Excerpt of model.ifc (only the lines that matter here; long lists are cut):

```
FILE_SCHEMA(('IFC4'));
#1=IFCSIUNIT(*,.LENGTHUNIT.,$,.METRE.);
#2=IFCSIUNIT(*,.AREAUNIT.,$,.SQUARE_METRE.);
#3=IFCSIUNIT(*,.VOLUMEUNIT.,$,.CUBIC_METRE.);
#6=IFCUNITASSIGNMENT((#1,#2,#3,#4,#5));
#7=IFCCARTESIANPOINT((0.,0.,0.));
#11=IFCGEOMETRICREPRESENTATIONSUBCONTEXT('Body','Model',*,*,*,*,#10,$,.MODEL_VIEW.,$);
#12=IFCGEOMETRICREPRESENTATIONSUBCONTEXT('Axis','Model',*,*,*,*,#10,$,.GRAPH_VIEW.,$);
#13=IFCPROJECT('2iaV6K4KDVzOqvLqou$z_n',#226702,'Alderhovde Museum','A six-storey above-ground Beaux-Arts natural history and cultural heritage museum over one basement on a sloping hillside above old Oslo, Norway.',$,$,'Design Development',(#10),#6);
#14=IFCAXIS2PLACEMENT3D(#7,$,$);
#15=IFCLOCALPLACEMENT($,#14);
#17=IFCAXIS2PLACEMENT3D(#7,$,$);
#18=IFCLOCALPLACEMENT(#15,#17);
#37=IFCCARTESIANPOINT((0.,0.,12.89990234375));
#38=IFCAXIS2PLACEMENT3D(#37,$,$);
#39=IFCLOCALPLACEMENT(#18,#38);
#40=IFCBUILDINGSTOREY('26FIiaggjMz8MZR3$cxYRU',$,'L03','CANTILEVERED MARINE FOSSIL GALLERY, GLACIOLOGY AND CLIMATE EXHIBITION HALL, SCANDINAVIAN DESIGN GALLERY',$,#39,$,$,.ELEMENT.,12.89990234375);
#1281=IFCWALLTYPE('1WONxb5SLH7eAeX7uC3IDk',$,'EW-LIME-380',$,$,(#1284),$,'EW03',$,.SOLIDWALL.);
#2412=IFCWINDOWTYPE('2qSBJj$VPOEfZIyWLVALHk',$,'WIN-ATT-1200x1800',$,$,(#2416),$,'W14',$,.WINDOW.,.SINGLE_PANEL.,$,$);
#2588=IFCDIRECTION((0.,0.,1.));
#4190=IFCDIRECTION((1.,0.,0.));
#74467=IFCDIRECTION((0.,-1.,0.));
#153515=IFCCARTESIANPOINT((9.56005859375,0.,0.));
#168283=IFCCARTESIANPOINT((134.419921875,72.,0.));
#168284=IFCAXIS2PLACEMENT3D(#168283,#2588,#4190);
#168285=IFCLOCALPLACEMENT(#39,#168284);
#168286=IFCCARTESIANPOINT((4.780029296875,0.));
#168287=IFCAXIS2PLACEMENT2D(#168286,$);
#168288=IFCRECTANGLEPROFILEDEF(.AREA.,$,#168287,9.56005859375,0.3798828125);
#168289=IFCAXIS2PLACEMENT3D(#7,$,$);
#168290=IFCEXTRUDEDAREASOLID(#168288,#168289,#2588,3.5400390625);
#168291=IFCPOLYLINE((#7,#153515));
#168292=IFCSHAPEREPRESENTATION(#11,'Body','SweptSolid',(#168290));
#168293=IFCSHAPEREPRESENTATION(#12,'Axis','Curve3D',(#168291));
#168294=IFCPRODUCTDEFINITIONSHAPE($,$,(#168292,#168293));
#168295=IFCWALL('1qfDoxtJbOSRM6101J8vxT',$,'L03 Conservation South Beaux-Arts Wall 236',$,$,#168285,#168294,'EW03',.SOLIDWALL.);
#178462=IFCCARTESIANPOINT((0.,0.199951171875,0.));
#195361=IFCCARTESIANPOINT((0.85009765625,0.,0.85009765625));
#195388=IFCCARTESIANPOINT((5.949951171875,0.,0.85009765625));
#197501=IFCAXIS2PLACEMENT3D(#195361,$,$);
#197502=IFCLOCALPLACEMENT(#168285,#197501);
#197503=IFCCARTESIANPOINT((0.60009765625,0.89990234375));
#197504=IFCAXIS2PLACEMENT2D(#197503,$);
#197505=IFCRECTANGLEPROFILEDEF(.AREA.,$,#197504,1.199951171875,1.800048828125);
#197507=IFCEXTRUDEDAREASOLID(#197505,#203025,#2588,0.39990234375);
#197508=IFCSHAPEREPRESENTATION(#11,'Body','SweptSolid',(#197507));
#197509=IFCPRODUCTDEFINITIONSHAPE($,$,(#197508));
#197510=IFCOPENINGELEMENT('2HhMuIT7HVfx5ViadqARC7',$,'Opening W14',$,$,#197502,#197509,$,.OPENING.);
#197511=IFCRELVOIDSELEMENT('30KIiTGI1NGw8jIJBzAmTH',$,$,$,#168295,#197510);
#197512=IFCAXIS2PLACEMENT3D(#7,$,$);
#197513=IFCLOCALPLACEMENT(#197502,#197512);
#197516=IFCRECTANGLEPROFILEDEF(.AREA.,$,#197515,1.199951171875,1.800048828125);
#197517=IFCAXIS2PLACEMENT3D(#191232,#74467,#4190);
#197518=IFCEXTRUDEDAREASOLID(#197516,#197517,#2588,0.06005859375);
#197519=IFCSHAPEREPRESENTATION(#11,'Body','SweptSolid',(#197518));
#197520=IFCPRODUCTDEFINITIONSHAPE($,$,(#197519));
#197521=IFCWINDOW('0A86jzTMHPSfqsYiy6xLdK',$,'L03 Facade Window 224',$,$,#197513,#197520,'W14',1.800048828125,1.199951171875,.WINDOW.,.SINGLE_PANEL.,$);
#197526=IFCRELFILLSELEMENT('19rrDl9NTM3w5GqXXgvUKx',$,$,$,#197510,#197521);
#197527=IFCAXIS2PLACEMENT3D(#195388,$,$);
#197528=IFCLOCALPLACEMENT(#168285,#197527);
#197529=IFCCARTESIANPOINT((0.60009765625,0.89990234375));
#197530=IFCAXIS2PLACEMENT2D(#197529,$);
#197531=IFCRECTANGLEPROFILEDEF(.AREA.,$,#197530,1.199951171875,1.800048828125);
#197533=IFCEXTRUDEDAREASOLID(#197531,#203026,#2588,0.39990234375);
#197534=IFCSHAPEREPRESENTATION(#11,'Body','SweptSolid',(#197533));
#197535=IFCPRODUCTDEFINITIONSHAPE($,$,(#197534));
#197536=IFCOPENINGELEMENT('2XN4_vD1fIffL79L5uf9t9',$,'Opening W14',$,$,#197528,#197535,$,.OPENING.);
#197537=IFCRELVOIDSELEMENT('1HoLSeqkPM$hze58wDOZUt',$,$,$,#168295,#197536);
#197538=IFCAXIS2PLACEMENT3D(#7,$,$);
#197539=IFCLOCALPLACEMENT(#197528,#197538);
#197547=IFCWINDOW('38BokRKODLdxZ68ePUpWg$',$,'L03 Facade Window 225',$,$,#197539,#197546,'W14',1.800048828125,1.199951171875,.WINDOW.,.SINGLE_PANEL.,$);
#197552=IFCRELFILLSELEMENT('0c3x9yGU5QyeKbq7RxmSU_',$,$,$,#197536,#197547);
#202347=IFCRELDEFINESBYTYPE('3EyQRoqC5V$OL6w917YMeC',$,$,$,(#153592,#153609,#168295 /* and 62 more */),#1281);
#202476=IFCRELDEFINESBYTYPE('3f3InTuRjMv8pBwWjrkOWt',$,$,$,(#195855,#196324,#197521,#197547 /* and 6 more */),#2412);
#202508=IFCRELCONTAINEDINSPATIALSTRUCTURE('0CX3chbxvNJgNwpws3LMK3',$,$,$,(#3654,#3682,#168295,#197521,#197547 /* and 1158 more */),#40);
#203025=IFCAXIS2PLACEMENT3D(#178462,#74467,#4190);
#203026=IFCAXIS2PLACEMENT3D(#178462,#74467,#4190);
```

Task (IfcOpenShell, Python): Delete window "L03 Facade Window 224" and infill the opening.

```python
import ifcopenshell
import ifcopenshell.api.feature
import ifcopenshell.api.root
import ifcopenshell.geom
import ifcopenshell.util.shape

model = ifcopenshell.open("model.ifc")
settings = ifcopenshell.geom.settings()


def volume(element):
    """Net volume in cubic metres, openings subtracted."""
    shape = ifcopenshell.geom.create_shape(settings, element)
    return ifcopenshell.util.shape.get_volume(shape.geometry)


window = model.by_guid("0A86jzTMHPSfqsYiy6xLdK")
opening = window.FillsVoids[0].RelatingOpeningElement
wall = opening.VoidsElements[0].RelatingBuildingElement
before = volume(wall)

ifcopenshell.api.root.remove_product(model, product=window)
ifcopenshell.api.feature.remove_feature(model, feature=opening)

after = volume(wall)

print(f"wall volume {before:.3f} -> {after:.3f} m3")

model.write("model_v2.ifc")
```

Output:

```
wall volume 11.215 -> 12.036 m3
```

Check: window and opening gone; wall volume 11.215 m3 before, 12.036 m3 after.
